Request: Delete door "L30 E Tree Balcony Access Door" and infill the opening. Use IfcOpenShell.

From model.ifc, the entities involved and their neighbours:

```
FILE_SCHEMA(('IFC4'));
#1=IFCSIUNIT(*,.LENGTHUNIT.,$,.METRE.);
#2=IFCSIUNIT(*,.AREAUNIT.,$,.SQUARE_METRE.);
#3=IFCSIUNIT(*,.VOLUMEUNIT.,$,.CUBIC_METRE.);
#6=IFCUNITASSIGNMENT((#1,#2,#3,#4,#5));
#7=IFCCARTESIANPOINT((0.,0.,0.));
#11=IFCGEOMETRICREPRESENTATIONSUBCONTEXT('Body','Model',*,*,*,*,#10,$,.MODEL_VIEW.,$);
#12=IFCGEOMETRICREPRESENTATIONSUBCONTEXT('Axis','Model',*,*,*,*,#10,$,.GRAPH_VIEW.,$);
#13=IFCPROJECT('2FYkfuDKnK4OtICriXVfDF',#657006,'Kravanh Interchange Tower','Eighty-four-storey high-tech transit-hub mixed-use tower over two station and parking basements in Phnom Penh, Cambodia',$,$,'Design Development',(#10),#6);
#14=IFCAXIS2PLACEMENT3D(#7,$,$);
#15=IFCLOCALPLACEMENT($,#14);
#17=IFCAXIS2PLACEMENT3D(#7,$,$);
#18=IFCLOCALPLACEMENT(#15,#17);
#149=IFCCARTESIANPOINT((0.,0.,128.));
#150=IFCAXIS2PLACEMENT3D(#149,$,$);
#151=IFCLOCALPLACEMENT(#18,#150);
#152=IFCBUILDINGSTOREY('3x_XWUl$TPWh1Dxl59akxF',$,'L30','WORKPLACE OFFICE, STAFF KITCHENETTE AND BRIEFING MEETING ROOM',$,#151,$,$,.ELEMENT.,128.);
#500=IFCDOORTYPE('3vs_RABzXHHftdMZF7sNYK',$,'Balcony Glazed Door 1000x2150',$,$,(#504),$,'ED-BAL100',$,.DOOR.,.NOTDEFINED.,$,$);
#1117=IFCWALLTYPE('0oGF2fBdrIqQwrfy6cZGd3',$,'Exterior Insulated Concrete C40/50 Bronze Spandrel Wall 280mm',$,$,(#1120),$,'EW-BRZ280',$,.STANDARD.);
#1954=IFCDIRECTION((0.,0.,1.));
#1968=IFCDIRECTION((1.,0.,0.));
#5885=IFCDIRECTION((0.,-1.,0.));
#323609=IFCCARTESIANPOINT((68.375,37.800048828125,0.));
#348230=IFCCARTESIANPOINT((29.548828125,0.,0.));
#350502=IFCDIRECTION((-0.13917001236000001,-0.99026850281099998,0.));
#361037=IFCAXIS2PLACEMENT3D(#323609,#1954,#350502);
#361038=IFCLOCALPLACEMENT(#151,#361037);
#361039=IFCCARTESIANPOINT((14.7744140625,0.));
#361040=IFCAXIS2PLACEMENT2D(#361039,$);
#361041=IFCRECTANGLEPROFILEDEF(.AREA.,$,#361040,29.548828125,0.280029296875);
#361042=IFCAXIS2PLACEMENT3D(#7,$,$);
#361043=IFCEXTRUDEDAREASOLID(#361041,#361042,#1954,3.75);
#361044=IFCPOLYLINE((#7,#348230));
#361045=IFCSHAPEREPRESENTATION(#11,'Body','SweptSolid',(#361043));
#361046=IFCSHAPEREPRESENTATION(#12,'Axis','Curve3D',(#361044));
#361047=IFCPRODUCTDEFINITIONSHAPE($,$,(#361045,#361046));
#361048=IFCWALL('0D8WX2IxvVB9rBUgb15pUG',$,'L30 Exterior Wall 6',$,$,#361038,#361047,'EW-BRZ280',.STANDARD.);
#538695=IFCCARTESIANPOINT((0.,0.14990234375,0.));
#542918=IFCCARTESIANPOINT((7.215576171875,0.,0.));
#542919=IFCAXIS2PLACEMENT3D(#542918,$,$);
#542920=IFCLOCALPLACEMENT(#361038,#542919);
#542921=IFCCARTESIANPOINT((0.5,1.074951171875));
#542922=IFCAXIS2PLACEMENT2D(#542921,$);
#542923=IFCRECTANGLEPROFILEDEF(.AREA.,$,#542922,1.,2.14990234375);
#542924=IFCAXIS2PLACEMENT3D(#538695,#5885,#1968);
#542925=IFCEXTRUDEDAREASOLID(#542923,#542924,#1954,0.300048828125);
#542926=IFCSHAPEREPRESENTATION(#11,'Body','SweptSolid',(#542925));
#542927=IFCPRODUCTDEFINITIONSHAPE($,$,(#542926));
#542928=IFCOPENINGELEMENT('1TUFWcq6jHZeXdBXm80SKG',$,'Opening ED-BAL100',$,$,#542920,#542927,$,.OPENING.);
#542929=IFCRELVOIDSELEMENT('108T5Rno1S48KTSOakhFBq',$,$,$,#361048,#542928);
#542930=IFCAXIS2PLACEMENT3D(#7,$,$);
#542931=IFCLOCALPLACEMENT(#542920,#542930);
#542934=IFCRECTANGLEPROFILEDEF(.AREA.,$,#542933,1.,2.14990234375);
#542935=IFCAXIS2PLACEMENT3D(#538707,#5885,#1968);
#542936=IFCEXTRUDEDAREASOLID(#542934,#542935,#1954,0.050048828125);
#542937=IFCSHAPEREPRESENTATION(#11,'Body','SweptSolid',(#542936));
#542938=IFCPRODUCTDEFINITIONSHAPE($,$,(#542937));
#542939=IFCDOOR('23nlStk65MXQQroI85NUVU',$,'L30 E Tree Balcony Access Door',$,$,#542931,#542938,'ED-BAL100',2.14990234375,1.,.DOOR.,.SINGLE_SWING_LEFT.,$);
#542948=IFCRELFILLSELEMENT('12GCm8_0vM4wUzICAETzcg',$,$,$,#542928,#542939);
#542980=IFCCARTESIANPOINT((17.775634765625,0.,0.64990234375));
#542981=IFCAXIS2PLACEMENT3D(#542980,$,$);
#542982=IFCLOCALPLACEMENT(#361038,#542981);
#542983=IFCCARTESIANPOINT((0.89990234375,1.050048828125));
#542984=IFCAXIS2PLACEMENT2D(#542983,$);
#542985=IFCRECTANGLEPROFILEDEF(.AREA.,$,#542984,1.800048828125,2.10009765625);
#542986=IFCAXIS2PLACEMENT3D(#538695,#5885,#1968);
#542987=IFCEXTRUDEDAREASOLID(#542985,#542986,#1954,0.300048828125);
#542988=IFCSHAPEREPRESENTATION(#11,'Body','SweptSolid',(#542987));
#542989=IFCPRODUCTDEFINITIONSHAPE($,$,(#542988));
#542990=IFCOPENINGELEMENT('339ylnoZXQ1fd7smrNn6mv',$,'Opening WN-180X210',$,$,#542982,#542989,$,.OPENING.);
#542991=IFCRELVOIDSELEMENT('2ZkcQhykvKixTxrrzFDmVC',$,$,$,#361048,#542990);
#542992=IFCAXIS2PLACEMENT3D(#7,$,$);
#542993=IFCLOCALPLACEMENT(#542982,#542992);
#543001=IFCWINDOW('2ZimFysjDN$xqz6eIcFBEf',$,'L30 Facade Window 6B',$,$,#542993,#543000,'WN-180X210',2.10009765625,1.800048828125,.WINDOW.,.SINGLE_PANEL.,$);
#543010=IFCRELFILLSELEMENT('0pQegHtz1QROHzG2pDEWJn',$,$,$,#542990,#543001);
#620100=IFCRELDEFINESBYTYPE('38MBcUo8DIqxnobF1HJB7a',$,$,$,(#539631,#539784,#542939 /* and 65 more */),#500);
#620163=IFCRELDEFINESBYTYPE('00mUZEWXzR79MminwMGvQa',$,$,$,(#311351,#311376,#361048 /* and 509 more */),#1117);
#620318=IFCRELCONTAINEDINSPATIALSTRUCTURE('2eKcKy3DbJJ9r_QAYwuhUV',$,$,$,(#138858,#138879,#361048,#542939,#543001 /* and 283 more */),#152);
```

```python
import ifcopenshell
import ifcopenshell.api.feature
import ifcopenshell.api.root
import ifcopenshell.geom
import ifcopenshell.util.shape

model = ifcopenshell.open("model.ifc")
settings = ifcopenshell.geom.settings()


def volume(element):
    """Net volume in cubic metres, openings subtracted."""
    shape = ifcopenshell.geom.create_shape(settings, element)
    return ifcopenshell.util.shape.get_volume(shape.geometry)


door = model.by_guid("23nlStk65MXQQroI85NUVU")
opening = door.FillsVoids[0].RelatingOpeningElement
wall = opening.VoidsElements[0].RelatingBuildingElement
before = volume(wall)

ifcopenshell.api.root.remove_product(model, product=door)
ifcopenshell.api.feature.remove_feature(model, feature=opening)

after = volume(wall)

print(f"wall volume {before:.3f} -> {after:.3f} m3")

model.write("model_rev.ifc")
```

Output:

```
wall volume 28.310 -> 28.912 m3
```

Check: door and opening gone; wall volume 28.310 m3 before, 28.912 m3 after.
